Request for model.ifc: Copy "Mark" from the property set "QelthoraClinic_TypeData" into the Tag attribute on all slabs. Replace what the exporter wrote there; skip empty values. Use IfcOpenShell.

First a look at what the model holds.

```python
import ifcopenshell
import ifcopenshell.util.element

model = ifcopenshell.open("model.ifc")
print(model.schema)
slabs = model.by_type("IfcSlab")
print(len(slabs), "slabs")
for e in slabs[:8]:
    source = ifcopenshell.util.element.get_pset(e, "QelthoraClinic_TypeData", "Mark")
    target = e.Tag
    print(e.id(), repr(source), repr(target), sep=" | ")
```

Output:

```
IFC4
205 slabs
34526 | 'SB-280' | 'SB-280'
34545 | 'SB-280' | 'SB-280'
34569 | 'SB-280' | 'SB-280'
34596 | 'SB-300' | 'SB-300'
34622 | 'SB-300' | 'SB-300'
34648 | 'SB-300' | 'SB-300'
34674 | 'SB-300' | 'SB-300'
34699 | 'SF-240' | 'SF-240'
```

```python
import ifcopenshell
import ifcopenshell.util.element

model = ifcopenshell.open("model.ifc")

count = 0
for e in model.by_type("IfcSlab"):
    value = ifcopenshell.util.element.get_pset(e, "QelthoraClinic_TypeData", "Mark")
    current = e.Tag
    if not value or not value.strip() or current == value:
        continue
    e.Tag = value
    count += 1

print(count, "slabs updated")

model.write("model_updated.ifc")
```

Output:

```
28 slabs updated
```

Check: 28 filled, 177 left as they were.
